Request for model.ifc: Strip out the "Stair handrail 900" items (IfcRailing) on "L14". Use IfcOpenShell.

First a look at what the model holds.

```python
import ifcopenshell
import ifcopenshell.util.element

model = ifcopenshell.open("model.ifc")
print(model.schema)
storey = next(s for s in model.by_type("IfcBuildingStorey") if s.Name == "L14")
railings = [e for e in ifcopenshell.util.element.get_decomposition(storey) if e.is_a("IfcRailing")]
seen = {}
for e in railings:
    element_type = ifcopenshell.util.element.get_type(e)
    name = element_type.Name if element_type not in (None, e) else None
    seen[name] = seen.get(name, 0) + 1
for name, count in sorted(seen.items(), key=str):
    print(count, "x", name)
```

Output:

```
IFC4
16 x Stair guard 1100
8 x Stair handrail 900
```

```python
import ifcopenshell
import ifcopenshell.api.root
import ifcopenshell.util.element

model = ifcopenshell.open("model.ifc")

storey = next(s for s in model.by_type("IfcBuildingStorey") if s.Name == "L14")
railings = [e for e in ifcopenshell.util.element.get_decomposition(storey) if e.is_a("IfcRailing")]
targets = [e for e in railings if (t := ifcopenshell.util.element.get_type(e)) not in (None, e) and t.Name == "Stair handrail 900"]

for e in targets:
    ifcopenshell.api.root.remove_product(model, product=e)
print(len(targets), "removed")

model.write("model_edited.ifc")
```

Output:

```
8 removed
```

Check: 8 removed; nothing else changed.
